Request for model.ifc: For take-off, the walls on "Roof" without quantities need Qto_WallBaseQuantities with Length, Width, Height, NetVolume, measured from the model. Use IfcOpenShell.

First a look at what the model holds.

```python
import ifcopenshell
import ifcopenshell.util.element
import ifcopenshell.util.unit

model = ifcopenshell.open("model.ifc")
print(model.schema)
for unit_type in ("LENGTHUNIT", "AREAUNIT", "VOLUMEUNIT"):
    print(unit_type, ifcopenshell.util.unit.calculate_unit_scale(model, unit_type))
storey = next(s for s in model.by_type("IfcBuildingStorey") if s.Name == "Roof")
walls = [e for e in ifcopenshell.util.element.get_decomposition(storey) if e.is_a("IfcWall")]
for e in sorted(walls, key=lambda e: e.id()):
    print(e.id(), e.is_a(), e.Name, list(ifcopenshell.util.element.get_psets(e, qtos_only=True)), sep=" | ")
```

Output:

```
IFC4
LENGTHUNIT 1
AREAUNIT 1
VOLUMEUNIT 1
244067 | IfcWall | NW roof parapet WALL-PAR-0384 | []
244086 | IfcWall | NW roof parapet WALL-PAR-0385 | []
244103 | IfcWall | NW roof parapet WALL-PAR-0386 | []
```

```python
import ifcopenshell
import ifcopenshell.api.pset
import ifcopenshell.geom
import ifcopenshell.util.element
import ifcopenshell.util.shape
import ifcopenshell.util.unit

model = ifcopenshell.open("model.ifc")
unit_scale = ifcopenshell.util.unit.calculate_unit_scale(model)
volume_scale = ifcopenshell.util.unit.calculate_unit_scale(model, "VOLUMEUNIT")
settings = ifcopenshell.geom.settings()

storey = next(s for s in model.by_type("IfcBuildingStorey") if s.Name == "Roof")
walls = [e for e in ifcopenshell.util.element.get_decomposition(storey) if e.is_a("IfcWall")]

for e in sorted(walls, key=lambda e: e.id()):
    if ifcopenshell.util.element.get_psets(e, qtos_only=True, should_inherit=False):
        continue
    # Geometry comes back in metres, in the element's own axes.
    shape = ifcopenshell.geom.create_shape(settings, e)
    values = {
        "Length": ifcopenshell.util.shape.get_x(shape.geometry) / unit_scale,
        "Width": ifcopenshell.util.shape.get_y(shape.geometry) / unit_scale,
        "Height": ifcopenshell.util.shape.get_z(shape.geometry) / unit_scale,
        "NetVolume": ifcopenshell.util.shape.get_volume(shape.geometry) / volume_scale,
    }
    qto = ifcopenshell.api.pset.add_qto(model, product=e, name="Qto_WallBaseQuantities")
    ifcopenshell.api.pset.edit_qto(model, qto=qto, properties=values)
    print(e.id(), {k: round(v, 3) for k, v in values.items()})

model.write("model_edited.ifc")
```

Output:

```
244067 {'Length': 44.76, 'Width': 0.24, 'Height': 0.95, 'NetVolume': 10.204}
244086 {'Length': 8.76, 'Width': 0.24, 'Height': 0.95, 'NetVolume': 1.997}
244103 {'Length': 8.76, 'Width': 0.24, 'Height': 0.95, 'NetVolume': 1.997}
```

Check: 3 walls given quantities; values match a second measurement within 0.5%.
